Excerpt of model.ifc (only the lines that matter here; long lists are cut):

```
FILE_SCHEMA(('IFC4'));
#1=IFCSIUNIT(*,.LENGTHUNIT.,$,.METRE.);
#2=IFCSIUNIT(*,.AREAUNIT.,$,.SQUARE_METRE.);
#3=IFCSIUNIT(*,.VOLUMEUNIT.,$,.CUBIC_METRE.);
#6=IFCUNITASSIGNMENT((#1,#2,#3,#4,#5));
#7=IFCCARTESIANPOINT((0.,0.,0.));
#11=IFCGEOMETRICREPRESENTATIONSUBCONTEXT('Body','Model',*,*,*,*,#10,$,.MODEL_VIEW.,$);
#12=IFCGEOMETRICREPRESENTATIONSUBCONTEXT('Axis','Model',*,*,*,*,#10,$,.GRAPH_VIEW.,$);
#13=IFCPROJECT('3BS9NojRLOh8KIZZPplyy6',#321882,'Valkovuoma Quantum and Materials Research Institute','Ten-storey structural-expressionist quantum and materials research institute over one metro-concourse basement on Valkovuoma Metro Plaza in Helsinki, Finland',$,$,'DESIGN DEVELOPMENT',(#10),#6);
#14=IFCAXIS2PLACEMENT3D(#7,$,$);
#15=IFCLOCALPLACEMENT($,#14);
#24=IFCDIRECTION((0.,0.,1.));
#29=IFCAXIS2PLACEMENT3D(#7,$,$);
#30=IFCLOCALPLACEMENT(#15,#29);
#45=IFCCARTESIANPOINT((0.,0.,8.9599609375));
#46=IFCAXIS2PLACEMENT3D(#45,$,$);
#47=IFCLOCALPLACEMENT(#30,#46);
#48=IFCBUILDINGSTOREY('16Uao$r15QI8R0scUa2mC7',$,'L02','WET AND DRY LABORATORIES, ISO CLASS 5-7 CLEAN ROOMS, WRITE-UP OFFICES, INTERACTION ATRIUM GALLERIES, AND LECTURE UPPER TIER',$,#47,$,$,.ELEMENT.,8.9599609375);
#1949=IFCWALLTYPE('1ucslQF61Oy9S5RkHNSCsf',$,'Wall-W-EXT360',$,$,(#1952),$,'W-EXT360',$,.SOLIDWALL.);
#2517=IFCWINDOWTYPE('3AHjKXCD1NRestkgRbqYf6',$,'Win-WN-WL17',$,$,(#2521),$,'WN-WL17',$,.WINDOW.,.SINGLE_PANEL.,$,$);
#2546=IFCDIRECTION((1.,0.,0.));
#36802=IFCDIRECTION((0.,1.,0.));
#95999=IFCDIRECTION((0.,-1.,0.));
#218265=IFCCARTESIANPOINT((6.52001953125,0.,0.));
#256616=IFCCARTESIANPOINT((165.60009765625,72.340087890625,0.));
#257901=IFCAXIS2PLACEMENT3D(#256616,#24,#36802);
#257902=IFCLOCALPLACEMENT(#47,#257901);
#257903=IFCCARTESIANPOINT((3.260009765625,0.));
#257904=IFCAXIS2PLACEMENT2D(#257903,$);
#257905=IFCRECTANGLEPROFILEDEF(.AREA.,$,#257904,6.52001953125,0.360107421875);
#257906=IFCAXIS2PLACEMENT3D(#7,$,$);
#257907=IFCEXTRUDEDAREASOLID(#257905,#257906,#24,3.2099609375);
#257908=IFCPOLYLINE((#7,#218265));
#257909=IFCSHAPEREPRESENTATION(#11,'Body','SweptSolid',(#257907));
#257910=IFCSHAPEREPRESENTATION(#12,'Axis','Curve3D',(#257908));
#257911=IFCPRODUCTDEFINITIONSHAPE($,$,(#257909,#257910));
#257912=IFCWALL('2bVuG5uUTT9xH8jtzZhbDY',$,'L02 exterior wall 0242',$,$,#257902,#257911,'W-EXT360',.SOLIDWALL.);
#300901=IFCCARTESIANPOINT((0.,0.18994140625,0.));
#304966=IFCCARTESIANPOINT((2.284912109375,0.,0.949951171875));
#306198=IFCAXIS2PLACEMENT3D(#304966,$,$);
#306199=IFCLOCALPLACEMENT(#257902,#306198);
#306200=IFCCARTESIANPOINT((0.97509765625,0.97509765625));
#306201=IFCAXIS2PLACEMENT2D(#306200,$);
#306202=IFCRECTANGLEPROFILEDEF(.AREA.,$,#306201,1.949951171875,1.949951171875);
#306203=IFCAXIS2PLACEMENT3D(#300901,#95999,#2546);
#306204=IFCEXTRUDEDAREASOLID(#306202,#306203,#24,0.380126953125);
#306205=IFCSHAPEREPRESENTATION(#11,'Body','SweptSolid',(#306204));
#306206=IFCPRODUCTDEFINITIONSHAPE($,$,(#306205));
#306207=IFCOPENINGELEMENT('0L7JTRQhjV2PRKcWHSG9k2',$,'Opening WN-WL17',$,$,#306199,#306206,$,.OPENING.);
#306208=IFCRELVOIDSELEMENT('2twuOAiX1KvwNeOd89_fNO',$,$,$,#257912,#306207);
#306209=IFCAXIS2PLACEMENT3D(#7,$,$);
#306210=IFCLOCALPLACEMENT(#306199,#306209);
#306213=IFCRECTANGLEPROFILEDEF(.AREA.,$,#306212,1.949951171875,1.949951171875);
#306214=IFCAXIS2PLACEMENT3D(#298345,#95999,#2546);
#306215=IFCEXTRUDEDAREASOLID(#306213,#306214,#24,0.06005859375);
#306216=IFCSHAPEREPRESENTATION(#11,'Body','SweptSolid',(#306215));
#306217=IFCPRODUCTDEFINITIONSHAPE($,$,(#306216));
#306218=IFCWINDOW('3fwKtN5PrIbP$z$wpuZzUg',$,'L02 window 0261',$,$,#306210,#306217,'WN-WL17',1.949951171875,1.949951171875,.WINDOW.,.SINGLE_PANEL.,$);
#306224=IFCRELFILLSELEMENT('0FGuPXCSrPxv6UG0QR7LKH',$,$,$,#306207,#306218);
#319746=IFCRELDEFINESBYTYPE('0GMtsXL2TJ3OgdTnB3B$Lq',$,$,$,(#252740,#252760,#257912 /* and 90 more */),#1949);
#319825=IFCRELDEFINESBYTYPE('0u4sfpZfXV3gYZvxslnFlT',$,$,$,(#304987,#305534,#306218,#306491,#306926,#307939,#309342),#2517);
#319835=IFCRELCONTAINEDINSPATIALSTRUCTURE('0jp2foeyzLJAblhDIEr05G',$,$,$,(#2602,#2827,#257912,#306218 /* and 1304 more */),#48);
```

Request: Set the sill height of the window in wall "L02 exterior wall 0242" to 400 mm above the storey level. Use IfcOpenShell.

```python
import numpy as np
import ifcopenshell
import ifcopenshell.api.geometry
import ifcopenshell.geom
import ifcopenshell.util.element
import ifcopenshell.util.placement
import ifcopenshell.util.shape
import ifcopenshell.util.unit

model = ifcopenshell.open("model.ifc")
unit_scale = ifcopenshell.util.unit.calculate_unit_scale(model)

window = model.by_guid("3fwKtN5PrIbP$z$wpuZzUg")
opening = window.FillsVoids[0].RelatingOpeningElement
storey = ifcopenshell.util.element.get_container(window, ifc_class="IfcBuildingStorey")
level = ifcopenshell.util.placement.get_local_placement(storey.ObjectPlacement)[2, 3]

# The opening's origin need not be at the sill, so measure its lowest point.
shape = ifcopenshell.geom.create_shape(ifcopenshell.geom.settings(), opening)
bottom = ifcopenshell.util.shape.get_shape_bottom_elevation(shape, shape.geometry) / unit_scale
dz = level + 0.4 / unit_scale - bottom

shift = np.array([0.0, 0.0, dz])
# The window is placed relative to its opening, so it follows when the opening moves.
matrix = ifcopenshell.util.placement.get_local_placement(opening.ObjectPlacement)
matrix[:3, 3] += shift
ifcopenshell.api.geometry.edit_object_placement(
    model, product=opening, matrix=matrix, is_si=False, should_transform_children=True
)

print(f"moved by {dz * unit_scale:+.3f} m")

model.write("model_v2.ifc")
```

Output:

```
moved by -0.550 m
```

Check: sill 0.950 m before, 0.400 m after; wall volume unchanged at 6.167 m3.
